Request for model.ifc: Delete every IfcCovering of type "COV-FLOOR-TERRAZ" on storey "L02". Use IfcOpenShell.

First a look at what the model holds.

```python
import ifcopenshell
import ifcopenshell.util.element

model = ifcopenshell.open("model.ifc")
print(model.schema)
storey = next(s for s in model.by_type("IfcBuildingStorey") if s.Name == "L02")
coverings = [e for e in ifcopenshell.util.element.get_decomposition(storey) if e.is_a("IfcCovering")]
seen = {}
for e in coverings:
    element_type = ifcopenshell.util.element.get_type(e)
    name = element_type.Name if element_type not in (None, e) else None
    seen[name] = seen.get(name, 0) + 1
for name, count in sorted(seen.items(), key=str):
    print(count, "x", name)
```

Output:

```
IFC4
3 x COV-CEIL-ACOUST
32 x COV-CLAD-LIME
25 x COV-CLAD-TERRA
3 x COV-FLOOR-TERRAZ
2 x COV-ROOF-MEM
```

```python
import ifcopenshell
import ifcopenshell.api.root
import ifcopenshell.util.element

model = ifcopenshell.open("model.ifc")

storey = next(s for s in model.by_type("IfcBuildingStorey") if s.Name == "L02")
coverings = [e for e in ifcopenshell.util.element.get_decomposition(storey) if e.is_a("IfcCovering")]
targets = [e for e in coverings if (t := ifcopenshell.util.element.get_type(e)) not in (None, e) and t.Name == "COV-FLOOR-TERRAZ"]

for e in targets:
    ifcopenshell.api.root.remove_product(model, product=e)
print(len(targets), "removed")

model.write("model_v2.ifc")
```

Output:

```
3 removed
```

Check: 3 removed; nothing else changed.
